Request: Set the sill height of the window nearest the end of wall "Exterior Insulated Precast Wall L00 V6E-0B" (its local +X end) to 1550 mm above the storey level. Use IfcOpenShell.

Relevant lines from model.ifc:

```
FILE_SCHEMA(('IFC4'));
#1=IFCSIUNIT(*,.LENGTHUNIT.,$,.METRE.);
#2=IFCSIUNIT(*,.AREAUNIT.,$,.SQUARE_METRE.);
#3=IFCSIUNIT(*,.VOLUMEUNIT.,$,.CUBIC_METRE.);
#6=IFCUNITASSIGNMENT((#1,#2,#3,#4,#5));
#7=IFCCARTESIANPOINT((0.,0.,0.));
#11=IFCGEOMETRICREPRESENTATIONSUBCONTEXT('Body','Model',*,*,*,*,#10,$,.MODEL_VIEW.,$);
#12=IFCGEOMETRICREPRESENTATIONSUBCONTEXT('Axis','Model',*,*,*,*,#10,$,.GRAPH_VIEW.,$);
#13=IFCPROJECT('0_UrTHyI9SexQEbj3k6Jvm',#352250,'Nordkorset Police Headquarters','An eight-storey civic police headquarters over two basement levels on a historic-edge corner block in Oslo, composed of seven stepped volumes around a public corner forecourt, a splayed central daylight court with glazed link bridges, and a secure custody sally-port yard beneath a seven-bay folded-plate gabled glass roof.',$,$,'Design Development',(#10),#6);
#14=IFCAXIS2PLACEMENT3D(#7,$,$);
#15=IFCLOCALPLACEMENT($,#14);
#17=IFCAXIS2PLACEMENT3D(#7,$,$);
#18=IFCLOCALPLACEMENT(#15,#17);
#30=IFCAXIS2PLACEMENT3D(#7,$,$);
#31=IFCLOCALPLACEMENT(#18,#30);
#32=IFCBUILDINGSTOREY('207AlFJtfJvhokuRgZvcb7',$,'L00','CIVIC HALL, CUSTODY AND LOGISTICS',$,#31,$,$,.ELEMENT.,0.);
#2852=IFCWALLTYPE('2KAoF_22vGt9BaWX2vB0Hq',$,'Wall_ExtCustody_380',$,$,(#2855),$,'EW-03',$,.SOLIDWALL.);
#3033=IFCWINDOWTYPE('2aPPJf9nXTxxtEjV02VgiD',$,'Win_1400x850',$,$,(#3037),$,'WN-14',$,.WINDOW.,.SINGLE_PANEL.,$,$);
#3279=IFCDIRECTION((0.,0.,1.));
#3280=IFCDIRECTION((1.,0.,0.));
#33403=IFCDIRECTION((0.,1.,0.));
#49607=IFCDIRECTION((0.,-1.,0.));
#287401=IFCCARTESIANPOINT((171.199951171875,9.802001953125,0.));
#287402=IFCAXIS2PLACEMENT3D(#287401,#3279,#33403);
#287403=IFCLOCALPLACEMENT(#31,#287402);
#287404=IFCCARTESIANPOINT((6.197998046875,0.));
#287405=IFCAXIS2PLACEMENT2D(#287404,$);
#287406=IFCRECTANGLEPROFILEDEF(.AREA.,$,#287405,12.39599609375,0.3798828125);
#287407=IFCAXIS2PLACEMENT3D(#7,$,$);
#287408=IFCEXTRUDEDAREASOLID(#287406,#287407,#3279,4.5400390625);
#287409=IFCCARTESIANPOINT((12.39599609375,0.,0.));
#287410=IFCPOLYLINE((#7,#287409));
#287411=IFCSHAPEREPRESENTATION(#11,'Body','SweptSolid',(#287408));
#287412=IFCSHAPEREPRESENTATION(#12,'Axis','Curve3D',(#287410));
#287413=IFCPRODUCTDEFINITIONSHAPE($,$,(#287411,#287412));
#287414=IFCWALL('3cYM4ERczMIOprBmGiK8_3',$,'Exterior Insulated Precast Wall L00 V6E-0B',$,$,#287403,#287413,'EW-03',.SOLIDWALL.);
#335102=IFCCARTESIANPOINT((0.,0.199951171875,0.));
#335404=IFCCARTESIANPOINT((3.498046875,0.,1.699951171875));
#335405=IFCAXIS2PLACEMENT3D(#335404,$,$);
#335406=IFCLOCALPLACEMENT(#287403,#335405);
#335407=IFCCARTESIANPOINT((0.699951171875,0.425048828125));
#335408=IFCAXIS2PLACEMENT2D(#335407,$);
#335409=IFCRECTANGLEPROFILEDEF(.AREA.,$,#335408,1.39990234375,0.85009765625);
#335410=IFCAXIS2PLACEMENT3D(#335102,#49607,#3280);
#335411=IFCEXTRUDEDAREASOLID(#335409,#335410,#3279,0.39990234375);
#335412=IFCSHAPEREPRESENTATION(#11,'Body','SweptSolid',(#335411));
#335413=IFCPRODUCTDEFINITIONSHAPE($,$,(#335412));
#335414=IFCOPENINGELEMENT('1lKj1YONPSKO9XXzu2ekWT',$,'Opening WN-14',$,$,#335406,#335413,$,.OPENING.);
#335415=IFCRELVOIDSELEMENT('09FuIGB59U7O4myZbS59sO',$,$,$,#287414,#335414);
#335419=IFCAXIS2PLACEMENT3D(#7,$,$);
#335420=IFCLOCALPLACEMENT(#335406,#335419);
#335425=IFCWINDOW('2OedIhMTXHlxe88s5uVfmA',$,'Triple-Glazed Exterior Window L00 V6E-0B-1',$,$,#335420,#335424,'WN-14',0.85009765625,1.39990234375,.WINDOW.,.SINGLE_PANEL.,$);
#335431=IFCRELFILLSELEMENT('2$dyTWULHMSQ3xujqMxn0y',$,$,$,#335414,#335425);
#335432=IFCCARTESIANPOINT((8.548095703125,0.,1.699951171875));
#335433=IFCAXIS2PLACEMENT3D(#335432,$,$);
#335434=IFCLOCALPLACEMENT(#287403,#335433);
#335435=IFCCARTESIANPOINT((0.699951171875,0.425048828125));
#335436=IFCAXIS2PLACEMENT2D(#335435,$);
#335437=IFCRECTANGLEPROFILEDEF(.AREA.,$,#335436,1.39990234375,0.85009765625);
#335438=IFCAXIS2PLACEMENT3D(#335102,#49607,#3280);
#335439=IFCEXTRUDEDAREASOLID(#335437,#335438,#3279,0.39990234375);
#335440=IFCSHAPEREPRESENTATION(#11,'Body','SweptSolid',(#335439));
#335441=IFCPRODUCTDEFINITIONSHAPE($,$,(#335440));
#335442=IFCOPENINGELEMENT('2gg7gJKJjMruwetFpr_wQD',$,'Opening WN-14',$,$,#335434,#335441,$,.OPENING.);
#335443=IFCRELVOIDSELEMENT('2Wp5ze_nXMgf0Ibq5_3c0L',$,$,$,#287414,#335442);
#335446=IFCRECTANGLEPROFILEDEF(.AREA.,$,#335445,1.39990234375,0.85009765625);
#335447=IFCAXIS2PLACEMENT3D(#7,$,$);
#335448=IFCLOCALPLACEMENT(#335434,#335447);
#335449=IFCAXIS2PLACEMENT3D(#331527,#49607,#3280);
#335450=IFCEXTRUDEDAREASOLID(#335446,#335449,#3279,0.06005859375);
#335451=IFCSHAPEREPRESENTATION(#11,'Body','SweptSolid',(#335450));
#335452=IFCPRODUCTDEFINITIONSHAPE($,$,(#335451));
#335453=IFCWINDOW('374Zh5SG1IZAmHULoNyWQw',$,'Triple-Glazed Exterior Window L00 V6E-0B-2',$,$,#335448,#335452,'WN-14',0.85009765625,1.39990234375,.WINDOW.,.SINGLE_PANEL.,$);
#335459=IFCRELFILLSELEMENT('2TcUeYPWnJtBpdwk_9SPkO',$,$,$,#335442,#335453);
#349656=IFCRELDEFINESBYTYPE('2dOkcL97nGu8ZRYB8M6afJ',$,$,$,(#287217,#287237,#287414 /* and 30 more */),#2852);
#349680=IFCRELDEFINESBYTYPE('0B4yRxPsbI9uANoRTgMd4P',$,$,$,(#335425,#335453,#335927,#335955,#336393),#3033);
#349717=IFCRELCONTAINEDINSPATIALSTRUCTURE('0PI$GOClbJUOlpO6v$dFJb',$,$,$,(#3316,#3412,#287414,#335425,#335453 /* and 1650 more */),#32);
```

```python
import numpy as np
import ifcopenshell
import ifcopenshell.api.geometry
import ifcopenshell.geom
import ifcopenshell.util.element
import ifcopenshell.util.placement
import ifcopenshell.util.shape
import ifcopenshell.util.unit

model = ifcopenshell.open("model.ifc")
unit_scale = ifcopenshell.util.unit.calculate_unit_scale(model)

window = model.by_guid("374Zh5SG1IZAmHULoNyWQw")
opening = window.FillsVoids[0].RelatingOpeningElement
storey = ifcopenshell.util.element.get_container(window, ifc_class="IfcBuildingStorey")
level = ifcopenshell.util.placement.get_local_placement(storey.ObjectPlacement)[2, 3]

# The opening's origin need not be at the sill, so measure its lowest point.
shape = ifcopenshell.geom.create_shape(ifcopenshell.geom.settings(), opening)
bottom = ifcopenshell.util.shape.get_shape_bottom_elevation(shape, shape.geometry) / unit_scale
dz = level + 1.55 / unit_scale - bottom

shift = np.array([0.0, 0.0, dz])
# The window is placed relative to its opening, so it follows when the opening moves.
matrix = ifcopenshell.util.placement.get_local_placement(opening.ObjectPlacement)
matrix[:3, 3] += shift
ifcopenshell.api.geometry.edit_object_placement(
    model, product=opening, matrix=matrix, is_si=False, should_transform_children=True
)

print(f"moved by {dz * unit_scale:+.3f} m")

model.write("model-out.ifc")
```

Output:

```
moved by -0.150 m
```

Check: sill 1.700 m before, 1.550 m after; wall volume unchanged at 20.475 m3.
